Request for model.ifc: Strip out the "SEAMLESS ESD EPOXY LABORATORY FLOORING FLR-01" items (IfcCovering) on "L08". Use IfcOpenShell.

First a look at what the model holds.

```python
import ifcopenshell
import ifcopenshell.util.element

model = ifcopenshell.open("model.ifc")
print(model.schema)
storey = next(s for s in model.by_type("IfcBuildingStorey") if s.Name == "L08")
coverings = [e for e in ifcopenshell.util.element.get_decomposition(storey) if e.is_a("IfcCovering")]
seen = {}
for e in coverings:
    element_type = ifcopenshell.util.element.get_type(e)
    name = element_type.Name if element_type not in (None, e) else None
    seen[name] = seen.get(name, 0) + 1
for name, count in sorted(seen.items(), key=str):
    print(count, "x", name)
```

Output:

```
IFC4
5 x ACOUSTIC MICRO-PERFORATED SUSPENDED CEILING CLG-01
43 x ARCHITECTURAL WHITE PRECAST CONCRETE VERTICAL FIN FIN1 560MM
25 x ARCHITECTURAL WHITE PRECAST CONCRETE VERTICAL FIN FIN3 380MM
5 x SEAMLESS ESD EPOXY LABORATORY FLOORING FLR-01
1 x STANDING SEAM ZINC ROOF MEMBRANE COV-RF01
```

```python
import ifcopenshell
import ifcopenshell.api.root
import ifcopenshell.util.element

model = ifcopenshell.open("model.ifc")

storey = next(s for s in model.by_type("IfcBuildingStorey") if s.Name == "L08")
coverings = [e for e in ifcopenshell.util.element.get_decomposition(storey) if e.is_a("IfcCovering")]
targets = [e for e in coverings if (t := ifcopenshell.util.element.get_type(e)) not in (None, e) and t.Name == "SEAMLESS ESD EPOXY LABORATORY FLOORING FLR-01"]

for e in targets:
    ifcopenshell.api.root.remove_product(model, product=e)
print(len(targets), "removed")

model.write("model_rev.ifc")
```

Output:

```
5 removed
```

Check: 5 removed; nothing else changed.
